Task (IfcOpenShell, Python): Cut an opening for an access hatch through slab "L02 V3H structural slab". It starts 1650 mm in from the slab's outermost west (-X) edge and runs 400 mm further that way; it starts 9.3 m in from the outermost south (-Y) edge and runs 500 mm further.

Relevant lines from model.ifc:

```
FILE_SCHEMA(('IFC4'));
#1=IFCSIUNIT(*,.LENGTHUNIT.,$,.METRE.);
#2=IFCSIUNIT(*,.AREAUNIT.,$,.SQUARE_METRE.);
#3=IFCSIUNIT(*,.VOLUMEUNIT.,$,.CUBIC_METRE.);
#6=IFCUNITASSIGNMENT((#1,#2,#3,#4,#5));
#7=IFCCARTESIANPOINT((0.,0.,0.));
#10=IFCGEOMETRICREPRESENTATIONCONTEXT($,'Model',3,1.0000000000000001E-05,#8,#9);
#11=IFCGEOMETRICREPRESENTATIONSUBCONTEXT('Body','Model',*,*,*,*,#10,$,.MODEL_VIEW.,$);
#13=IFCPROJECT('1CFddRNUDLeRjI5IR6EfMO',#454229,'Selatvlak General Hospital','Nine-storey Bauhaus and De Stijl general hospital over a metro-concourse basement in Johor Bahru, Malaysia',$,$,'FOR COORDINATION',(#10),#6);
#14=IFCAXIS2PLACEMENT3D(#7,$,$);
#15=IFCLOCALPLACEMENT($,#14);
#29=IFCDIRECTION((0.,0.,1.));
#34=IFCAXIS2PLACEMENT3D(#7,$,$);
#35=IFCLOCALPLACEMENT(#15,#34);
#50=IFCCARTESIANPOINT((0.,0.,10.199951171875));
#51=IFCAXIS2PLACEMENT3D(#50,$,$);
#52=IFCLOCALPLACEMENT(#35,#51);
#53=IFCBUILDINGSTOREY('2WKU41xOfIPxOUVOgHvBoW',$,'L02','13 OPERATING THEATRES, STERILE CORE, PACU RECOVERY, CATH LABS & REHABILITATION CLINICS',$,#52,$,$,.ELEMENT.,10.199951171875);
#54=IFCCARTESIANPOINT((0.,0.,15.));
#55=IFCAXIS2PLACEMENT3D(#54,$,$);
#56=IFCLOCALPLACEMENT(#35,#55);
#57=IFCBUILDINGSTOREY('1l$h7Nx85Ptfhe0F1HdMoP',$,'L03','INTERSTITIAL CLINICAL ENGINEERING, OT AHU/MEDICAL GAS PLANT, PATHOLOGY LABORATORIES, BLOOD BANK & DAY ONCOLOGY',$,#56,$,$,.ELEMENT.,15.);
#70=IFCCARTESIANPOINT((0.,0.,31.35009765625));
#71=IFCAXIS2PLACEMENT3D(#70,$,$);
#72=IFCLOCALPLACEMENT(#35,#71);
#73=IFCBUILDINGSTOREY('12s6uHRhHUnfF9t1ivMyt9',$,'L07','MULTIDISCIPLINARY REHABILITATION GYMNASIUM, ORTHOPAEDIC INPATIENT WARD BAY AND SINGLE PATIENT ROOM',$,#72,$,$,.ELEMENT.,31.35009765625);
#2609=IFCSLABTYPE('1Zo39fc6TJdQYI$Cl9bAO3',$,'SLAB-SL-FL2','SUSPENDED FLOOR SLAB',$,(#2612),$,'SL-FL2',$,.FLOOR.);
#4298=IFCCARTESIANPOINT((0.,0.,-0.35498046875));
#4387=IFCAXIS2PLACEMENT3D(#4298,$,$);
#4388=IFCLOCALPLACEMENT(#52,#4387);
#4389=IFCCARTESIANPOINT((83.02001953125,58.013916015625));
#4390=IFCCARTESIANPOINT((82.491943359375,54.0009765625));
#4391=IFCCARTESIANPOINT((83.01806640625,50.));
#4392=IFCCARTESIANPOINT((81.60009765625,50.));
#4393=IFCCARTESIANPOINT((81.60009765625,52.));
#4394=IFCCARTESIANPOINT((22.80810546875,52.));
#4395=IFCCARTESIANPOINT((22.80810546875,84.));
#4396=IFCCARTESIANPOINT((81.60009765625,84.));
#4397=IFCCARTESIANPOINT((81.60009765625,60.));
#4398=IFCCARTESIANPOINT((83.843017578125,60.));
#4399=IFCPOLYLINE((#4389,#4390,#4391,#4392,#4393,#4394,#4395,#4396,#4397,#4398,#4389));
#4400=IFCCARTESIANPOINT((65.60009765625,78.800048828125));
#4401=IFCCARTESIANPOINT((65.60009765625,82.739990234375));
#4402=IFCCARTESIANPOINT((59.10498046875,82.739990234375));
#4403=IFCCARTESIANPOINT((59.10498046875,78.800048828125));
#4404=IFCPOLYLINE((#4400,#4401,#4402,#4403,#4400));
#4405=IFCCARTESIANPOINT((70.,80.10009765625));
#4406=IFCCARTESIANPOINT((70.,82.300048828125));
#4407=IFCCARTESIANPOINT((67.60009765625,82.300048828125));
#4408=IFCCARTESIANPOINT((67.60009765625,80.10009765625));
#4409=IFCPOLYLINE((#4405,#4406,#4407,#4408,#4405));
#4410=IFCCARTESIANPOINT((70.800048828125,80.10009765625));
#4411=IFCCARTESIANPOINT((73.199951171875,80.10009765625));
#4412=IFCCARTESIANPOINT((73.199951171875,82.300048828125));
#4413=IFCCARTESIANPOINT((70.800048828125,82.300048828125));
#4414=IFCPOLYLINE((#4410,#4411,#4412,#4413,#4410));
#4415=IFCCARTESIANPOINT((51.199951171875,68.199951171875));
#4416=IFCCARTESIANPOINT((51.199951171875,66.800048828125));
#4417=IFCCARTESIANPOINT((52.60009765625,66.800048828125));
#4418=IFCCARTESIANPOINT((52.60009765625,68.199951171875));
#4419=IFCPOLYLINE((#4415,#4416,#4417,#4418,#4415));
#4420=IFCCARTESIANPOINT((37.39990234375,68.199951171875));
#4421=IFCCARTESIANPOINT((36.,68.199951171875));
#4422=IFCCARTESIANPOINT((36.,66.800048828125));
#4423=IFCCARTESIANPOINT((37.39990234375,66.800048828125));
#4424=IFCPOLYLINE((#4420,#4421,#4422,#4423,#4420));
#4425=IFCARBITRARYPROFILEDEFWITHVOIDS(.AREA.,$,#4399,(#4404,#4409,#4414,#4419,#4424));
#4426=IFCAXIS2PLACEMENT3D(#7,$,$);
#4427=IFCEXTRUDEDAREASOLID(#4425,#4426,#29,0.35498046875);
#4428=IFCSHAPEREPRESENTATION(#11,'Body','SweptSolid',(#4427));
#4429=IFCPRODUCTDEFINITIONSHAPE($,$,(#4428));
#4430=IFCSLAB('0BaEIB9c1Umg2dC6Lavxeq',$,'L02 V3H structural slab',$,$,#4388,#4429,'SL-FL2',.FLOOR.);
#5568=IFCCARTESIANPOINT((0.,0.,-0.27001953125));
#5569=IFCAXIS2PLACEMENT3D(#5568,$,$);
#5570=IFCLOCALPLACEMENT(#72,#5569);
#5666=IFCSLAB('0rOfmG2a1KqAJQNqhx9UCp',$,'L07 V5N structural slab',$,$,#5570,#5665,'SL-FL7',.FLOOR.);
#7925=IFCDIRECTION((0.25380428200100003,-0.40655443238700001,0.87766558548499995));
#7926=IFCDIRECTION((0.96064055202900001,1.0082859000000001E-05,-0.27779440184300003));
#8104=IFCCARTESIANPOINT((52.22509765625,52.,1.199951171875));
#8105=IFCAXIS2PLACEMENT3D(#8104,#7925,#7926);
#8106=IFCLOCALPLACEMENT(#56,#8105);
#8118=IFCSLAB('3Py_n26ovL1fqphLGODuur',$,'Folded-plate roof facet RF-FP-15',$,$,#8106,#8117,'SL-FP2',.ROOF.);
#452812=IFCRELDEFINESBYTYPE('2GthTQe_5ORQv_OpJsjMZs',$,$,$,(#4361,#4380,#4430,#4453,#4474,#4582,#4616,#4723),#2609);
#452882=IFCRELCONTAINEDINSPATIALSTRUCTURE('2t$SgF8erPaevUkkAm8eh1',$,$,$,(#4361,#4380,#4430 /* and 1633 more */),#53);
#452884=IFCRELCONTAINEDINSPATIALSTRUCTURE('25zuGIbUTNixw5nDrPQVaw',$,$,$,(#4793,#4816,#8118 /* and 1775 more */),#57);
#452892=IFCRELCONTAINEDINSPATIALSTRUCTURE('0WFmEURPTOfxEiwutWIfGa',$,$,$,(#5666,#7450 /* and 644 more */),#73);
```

```python
import numpy as np
import ifcopenshell
import ifcopenshell.api.feature
import ifcopenshell.api.geometry
import ifcopenshell.api.root
import ifcopenshell.geom
import ifcopenshell.util.placement
import ifcopenshell.util.representation
import ifcopenshell.util.shape
import ifcopenshell.util.unit

model = ifcopenshell.open("model.ifc")
unit_scale = ifcopenshell.util.unit.calculate_unit_scale(model)
settings = ifcopenshell.geom.settings()


def volume(element):
    """Net volume in cubic metres, openings subtracted."""
    shape = ifcopenshell.geom.create_shape(settings, element)
    return ifcopenshell.util.shape.get_volume(shape.geometry)


slab = model.by_guid("0BaEIB9c1Umg2dC6Lavxeq")
before = volume(slab)

# Extent in the slab's own axes, in metres. The edges named are its -X and -Y sides.
slab_shape = ifcopenshell.geom.create_shape(settings, slab)
vertices = ifcopenshell.util.shape.get_vertices(slab_shape.geometry)
x_min, y_min, bottom = vertices.min(axis=0)
top = vertices[:, 2].max()

opening = ifcopenshell.api.root.create_entity(model, ifc_class="IfcOpeningElement", name="Access hatch opening", predefined_type="OPENING")
context = ifcopenshell.util.representation.get_context(model, "Model", "Body", "MODEL_VIEW")
width, depth = 0.4, 0.5
outline = [(0.0, 0.0), (width, 0.0), (width, depth), (0.0, depth), (0.0, 0.0)]
# Overshoot both faces by 50 mm so the cut is clean.
shape = ifcopenshell.api.geometry.add_slab_representation(
    model, context=context, depth=top - bottom + 0.1, polyline=outline
)
ifcopenshell.api.geometry.assign_representation(model, product=opening, representation=shape)

matrix = ifcopenshell.util.placement.get_local_placement(slab.ObjectPlacement)
matrix[:, 3] = matrix @ np.append(np.array([x_min + 1.65, y_min + 9.3, bottom - 0.05]) / unit_scale, 1.0)
ifcopenshell.api.geometry.edit_object_placement(model, product=opening, matrix=matrix, is_si=False)
ifcopenshell.api.feature.add_feature(model, feature=opening, element=slab)

after = volume(slab)

print(f"slab volume {before:.3f} -> {after:.3f} m3")

model.write("model-out.ifc")
```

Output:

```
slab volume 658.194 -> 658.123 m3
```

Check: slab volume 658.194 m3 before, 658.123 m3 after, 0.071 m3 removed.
